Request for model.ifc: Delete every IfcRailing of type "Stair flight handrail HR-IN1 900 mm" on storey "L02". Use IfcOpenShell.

First a look at what the model holds.

```python
import ifcopenshell
import ifcopenshell.util.element

model = ifcopenshell.open("model.ifc")
print(model.schema)
storey = next(s for s in model.by_type("IfcBuildingStorey") if s.Name == "L02")
railings = [e for e in ifcopenshell.util.element.get_decomposition(storey) if e.is_a("IfcRailing")]
seen = {}
for e in railings:
    element_type = ifcopenshell.util.element.get_type(e)
    name = element_type.Name if element_type not in (None, e) else None
    seen[name] = seen.get(name, 0) + 1
for name, count in sorted(seen.items(), key=str):
    print(count, "x", name)
```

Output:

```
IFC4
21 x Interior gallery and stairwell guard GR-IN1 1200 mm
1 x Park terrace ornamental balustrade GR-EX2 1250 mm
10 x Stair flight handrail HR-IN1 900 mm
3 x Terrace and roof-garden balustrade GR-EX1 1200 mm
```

```python
import ifcopenshell
import ifcopenshell.api.root
import ifcopenshell.util.element

model = ifcopenshell.open("model.ifc")

storey = next(s for s in model.by_type("IfcBuildingStorey") if s.Name == "L02")
railings = [e for e in ifcopenshell.util.element.get_decomposition(storey) if e.is_a("IfcRailing")]
targets = [e for e in railings if (t := ifcopenshell.util.element.get_type(e)) not in (None, e) and t.Name == "Stair flight handrail HR-IN1 900 mm"]

for e in targets:
    ifcopenshell.api.root.remove_product(model, product=e)
print(len(targets), "removed")

model.write("model_rev.ifc")
```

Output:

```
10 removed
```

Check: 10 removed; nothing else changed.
